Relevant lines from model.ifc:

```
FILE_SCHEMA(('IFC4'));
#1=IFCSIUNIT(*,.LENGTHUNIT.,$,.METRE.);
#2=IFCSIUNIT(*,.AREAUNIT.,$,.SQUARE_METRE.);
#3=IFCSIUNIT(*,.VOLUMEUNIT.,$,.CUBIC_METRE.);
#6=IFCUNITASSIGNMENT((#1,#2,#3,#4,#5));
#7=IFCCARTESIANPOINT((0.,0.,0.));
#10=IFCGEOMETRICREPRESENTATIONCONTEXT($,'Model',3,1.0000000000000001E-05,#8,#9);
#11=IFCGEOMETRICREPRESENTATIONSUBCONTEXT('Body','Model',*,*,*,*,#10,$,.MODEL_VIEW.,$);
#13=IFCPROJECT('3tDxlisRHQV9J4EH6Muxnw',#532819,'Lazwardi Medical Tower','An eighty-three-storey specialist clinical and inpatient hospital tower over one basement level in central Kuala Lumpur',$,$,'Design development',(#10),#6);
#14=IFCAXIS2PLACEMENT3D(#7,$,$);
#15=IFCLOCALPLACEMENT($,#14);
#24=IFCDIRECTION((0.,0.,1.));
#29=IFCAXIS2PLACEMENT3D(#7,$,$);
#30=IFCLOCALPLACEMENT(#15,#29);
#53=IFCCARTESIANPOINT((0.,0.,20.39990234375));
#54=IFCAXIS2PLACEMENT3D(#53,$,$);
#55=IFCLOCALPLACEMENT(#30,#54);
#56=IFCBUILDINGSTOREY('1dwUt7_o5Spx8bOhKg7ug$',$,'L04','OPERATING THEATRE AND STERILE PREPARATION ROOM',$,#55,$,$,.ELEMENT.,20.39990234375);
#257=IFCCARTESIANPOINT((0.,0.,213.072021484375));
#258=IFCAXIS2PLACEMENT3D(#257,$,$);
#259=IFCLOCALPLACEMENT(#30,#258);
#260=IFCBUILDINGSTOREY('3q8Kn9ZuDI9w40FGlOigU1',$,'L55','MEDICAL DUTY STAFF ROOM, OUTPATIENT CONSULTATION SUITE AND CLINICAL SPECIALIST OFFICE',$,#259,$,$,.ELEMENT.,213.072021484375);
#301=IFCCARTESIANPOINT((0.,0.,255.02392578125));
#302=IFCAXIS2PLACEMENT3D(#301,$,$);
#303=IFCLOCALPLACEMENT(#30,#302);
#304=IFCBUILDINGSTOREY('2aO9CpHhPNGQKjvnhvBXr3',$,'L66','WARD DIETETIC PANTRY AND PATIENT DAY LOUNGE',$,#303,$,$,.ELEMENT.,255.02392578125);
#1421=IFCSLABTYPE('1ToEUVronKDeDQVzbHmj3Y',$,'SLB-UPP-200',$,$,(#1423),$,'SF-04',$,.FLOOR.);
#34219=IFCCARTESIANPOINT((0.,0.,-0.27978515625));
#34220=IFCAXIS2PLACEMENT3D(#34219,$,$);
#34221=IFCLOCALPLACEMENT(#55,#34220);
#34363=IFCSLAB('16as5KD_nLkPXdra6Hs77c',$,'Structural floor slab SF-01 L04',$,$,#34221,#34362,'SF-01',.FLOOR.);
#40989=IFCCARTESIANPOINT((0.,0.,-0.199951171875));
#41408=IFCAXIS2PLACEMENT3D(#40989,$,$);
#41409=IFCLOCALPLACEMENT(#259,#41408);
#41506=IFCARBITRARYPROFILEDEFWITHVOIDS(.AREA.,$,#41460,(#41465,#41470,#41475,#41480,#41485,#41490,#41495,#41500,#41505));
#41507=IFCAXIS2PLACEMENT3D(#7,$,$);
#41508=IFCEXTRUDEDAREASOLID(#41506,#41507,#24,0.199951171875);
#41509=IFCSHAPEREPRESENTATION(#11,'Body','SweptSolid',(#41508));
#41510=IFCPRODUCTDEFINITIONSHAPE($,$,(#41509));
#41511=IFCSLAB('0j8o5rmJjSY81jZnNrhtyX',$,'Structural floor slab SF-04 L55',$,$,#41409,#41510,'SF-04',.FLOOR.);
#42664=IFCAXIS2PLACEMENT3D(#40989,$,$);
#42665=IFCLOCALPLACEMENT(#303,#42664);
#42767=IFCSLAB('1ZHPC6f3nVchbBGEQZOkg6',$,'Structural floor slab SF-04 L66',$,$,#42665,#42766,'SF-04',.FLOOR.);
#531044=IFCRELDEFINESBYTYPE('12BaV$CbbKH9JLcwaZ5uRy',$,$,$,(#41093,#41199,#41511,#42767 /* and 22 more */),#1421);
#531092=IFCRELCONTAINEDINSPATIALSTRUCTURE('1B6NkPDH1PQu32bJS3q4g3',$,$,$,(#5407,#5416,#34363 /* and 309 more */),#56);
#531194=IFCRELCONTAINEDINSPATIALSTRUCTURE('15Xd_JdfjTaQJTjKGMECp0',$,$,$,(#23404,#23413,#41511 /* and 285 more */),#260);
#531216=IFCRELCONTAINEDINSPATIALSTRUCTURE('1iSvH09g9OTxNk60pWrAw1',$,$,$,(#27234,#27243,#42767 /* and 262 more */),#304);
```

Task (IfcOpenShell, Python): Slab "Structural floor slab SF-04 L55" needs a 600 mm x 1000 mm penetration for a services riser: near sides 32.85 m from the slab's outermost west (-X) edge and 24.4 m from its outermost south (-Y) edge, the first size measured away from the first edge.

```python
import numpy as np
import ifcopenshell
import ifcopenshell.api.feature
import ifcopenshell.api.geometry
import ifcopenshell.api.root
import ifcopenshell.geom
import ifcopenshell.util.placement
import ifcopenshell.util.representation
import ifcopenshell.util.shape
import ifcopenshell.util.unit

model = ifcopenshell.open("model.ifc")
unit_scale = ifcopenshell.util.unit.calculate_unit_scale(model)
settings = ifcopenshell.geom.settings()


def volume(element):
    """Net volume in cubic metres, openings subtracted."""
    shape = ifcopenshell.geom.create_shape(settings, element)
    return ifcopenshell.util.shape.get_volume(shape.geometry)


slab = model.by_id(41511)
before = volume(slab)

# Extent in the slab's own axes, in metres. The edges named are its -X and -Y sides.
slab_shape = ifcopenshell.geom.create_shape(settings, slab)
vertices = ifcopenshell.util.shape.get_vertices(slab_shape.geometry)
x_min, y_min, bottom = vertices.min(axis=0)
top = vertices[:, 2].max()

opening = ifcopenshell.api.root.create_entity(model, ifc_class="IfcOpeningElement", name="Services riser opening", predefined_type="OPENING")
context = ifcopenshell.util.representation.get_context(model, "Model", "Body", "MODEL_VIEW")
width, depth = 0.6, 1
outline = [(0.0, 0.0), (width, 0.0), (width, depth), (0.0, depth), (0.0, 0.0)]
# Overshoot both faces by 50 mm so the cut is clean.
shape = ifcopenshell.api.geometry.add_slab_representation(
    model, context=context, depth=top - bottom + 0.1, polyline=outline
)
ifcopenshell.api.geometry.assign_representation(model, product=opening, representation=shape)

matrix = ifcopenshell.util.placement.get_local_placement(slab.ObjectPlacement)
matrix[:, 3] = matrix @ np.append(np.array([x_min + 32.85, y_min + 24.4, bottom - 0.05]) / unit_scale, 1.0)
ifcopenshell.api.geometry.edit_object_placement(model, product=opening, matrix=matrix, is_si=False)
ifcopenshell.api.feature.add_feature(model, feature=opening, element=slab)

after = volume(slab)

print(f"slab volume {before:.3f} -> {after:.3f} m3")

model.write("model_updated.ifc")
```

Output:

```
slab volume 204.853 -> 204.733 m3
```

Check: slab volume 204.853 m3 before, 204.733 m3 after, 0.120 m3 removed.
